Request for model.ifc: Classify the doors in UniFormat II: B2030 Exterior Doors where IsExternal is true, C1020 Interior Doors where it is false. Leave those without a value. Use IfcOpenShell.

First a look at what the model holds.

```python
import ifcopenshell
import ifcopenshell.util.element

model = ifcopenshell.open("model.ifc")
print(model.schema)
print("classifications:", [c.Name for c in model.by_type("IfcClassification")])
values = [ifcopenshell.util.element.get_pset(e, "Pset_DoorCommon", "IsExternal") for e in model.by_type("IfcDoor")]
for value in (True, False, None):
    print("IsExternal", value, values.count(value))
```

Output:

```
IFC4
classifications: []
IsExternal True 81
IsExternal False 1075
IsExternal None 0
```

```python
import ifcopenshell
import ifcopenshell.api.classification
import ifcopenshell.util.element

model = ifcopenshell.open("model.ifc")

system = ifcopenshell.api.classification.add_classification(model, classification="UniFormat II")

doors = model.by_type("IfcDoor")
external = {e: ifcopenshell.util.element.get_pset(e, "Pset_DoorCommon", "IsExternal") for e in doors}
for flag, code, name in ((True, "B2030", "Exterior Doors"), (False, "C1020", "Interior Doors")):
    products = [e for e in doors if external[e] is flag]
    ifcopenshell.api.classification.add_reference(
        model, products=products, classification=system, identification=code, name=name
    )
    print(code, len(products))

model.write("model-out.ifc")
```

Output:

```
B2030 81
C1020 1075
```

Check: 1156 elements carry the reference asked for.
